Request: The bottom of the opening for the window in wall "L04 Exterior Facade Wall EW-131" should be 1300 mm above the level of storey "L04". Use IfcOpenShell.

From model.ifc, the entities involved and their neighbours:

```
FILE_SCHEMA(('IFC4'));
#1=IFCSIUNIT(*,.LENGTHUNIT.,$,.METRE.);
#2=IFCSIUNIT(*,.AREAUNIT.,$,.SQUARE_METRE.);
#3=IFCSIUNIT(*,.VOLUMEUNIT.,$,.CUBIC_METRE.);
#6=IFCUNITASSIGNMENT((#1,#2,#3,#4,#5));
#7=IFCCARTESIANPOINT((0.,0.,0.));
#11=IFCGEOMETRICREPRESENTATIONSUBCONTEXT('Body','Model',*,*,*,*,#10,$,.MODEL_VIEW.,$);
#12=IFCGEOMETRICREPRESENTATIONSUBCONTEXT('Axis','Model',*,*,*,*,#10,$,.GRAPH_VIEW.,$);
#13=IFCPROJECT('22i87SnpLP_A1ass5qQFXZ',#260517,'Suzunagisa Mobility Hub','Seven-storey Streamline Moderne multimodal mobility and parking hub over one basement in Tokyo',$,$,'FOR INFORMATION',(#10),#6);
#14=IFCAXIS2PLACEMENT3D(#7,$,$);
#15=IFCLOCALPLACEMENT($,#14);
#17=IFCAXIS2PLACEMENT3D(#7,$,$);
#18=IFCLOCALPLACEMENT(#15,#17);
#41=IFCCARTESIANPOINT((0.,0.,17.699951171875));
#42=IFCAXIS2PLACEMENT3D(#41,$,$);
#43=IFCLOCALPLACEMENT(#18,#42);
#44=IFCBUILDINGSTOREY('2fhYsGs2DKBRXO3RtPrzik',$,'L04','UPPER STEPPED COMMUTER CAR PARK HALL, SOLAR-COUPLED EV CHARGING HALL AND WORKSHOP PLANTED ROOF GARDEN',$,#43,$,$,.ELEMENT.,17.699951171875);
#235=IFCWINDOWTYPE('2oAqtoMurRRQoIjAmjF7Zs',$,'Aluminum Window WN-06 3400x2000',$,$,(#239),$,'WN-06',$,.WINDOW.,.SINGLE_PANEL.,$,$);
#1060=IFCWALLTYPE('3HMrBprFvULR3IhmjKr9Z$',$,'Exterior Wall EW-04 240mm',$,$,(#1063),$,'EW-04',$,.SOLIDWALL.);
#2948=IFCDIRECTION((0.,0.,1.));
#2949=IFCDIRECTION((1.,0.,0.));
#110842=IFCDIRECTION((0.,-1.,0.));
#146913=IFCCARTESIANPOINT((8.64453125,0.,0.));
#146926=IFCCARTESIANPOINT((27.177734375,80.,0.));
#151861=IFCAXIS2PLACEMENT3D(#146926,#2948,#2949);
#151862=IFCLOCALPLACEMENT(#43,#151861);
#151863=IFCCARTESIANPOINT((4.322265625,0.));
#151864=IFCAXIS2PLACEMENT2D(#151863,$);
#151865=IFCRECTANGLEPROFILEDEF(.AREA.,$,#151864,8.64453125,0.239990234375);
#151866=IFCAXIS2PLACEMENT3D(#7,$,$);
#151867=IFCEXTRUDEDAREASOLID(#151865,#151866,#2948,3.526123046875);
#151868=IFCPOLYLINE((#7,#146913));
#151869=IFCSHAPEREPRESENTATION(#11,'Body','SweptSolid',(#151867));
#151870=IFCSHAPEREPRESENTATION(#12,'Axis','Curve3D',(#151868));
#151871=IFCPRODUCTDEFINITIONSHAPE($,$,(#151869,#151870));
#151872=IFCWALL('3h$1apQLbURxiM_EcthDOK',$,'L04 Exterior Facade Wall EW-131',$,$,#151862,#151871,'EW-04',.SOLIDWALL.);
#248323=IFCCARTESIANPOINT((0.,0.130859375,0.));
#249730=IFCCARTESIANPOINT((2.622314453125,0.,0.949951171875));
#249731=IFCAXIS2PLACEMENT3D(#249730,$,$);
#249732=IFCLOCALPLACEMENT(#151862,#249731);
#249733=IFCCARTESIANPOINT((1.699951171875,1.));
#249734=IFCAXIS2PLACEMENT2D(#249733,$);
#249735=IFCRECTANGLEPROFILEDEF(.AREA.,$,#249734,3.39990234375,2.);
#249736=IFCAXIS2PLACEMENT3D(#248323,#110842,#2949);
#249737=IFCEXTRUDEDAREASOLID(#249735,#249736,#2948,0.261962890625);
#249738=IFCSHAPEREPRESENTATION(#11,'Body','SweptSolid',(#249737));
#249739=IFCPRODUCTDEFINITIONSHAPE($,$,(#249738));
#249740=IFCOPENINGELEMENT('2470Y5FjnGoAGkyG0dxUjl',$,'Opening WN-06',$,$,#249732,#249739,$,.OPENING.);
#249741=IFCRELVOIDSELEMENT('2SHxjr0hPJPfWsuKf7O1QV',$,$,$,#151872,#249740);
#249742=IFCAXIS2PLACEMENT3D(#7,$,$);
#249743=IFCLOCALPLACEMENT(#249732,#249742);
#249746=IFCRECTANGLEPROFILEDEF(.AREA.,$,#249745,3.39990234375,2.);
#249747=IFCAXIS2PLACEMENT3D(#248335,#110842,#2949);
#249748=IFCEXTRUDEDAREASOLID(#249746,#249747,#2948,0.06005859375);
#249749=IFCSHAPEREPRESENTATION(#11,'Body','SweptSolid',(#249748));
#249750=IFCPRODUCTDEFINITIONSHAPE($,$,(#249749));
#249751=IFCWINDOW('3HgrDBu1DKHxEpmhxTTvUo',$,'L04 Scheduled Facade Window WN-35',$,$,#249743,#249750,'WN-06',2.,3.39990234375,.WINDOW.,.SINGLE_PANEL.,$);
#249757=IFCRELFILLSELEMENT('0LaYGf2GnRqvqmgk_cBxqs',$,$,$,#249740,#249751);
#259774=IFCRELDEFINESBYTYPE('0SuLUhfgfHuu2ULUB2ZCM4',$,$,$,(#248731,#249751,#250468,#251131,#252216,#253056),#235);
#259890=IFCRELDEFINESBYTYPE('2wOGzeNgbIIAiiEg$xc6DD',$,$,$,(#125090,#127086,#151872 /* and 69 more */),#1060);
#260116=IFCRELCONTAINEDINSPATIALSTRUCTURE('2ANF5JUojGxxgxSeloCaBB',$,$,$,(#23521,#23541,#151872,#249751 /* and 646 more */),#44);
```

```python
import numpy as np
import ifcopenshell
import ifcopenshell.api.geometry
import ifcopenshell.geom
import ifcopenshell.util.element
import ifcopenshell.util.placement
import ifcopenshell.util.shape
import ifcopenshell.util.unit

model = ifcopenshell.open("model.ifc")
unit_scale = ifcopenshell.util.unit.calculate_unit_scale(model)

window = model.by_guid("3HgrDBu1DKHxEpmhxTTvUo")
opening = window.FillsVoids[0].RelatingOpeningElement
storey = ifcopenshell.util.element.get_container(window, ifc_class="IfcBuildingStorey")
level = ifcopenshell.util.placement.get_local_placement(storey.ObjectPlacement)[2, 3]

# The opening's origin need not be at the sill, so measure its lowest point.
shape = ifcopenshell.geom.create_shape(ifcopenshell.geom.settings(), opening)
bottom = ifcopenshell.util.shape.get_shape_bottom_elevation(shape, shape.geometry) / unit_scale
dz = level + 1.3 / unit_scale - bottom

shift = np.array([0.0, 0.0, dz])
# The window is placed relative to its opening, so it follows when the opening moves.
matrix = ifcopenshell.util.placement.get_local_placement(opening.ObjectPlacement)
matrix[:3, 3] += shift
ifcopenshell.api.geometry.edit_object_placement(
    model, product=opening, matrix=matrix, is_si=False, should_transform_children=True
)

print(f"moved by {dz * unit_scale:+.3f} m")

model.write("model_edited.ifc")
```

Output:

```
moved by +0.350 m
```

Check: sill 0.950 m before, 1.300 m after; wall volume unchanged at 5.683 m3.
